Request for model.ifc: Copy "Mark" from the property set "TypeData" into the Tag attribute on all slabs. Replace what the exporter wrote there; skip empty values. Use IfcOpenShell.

First a look at what the model holds.

```python
import ifcopenshell
import ifcopenshell.util.element

model = ifcopenshell.open("model.ifc")
print(model.schema)
slabs = model.by_type("IfcSlab")
print(len(slabs), "slabs")
for e in slabs[:8]:
    source = ifcopenshell.util.element.get_pset(e, "TypeData", "Mark")
    target = e.Tag
    print(e.id(), repr(source), repr(target), sep=" | ")
```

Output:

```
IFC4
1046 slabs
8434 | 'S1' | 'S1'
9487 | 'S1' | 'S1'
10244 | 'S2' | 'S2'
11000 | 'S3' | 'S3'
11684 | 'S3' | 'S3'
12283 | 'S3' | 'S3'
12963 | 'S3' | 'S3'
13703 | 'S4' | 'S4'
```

```python
import ifcopenshell
import ifcopenshell.util.element

model = ifcopenshell.open("model.ifc")

count = 0
for e in model.by_type("IfcSlab"):
    value = ifcopenshell.util.element.get_pset(e, "TypeData", "Mark")
    current = e.Tag
    if not value or not value.strip() or current == value:
        continue
    e.Tag = value
    count += 1

print(count, "slabs updated")

model.write("model_v2.ifc")
```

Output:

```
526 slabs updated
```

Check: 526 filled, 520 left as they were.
